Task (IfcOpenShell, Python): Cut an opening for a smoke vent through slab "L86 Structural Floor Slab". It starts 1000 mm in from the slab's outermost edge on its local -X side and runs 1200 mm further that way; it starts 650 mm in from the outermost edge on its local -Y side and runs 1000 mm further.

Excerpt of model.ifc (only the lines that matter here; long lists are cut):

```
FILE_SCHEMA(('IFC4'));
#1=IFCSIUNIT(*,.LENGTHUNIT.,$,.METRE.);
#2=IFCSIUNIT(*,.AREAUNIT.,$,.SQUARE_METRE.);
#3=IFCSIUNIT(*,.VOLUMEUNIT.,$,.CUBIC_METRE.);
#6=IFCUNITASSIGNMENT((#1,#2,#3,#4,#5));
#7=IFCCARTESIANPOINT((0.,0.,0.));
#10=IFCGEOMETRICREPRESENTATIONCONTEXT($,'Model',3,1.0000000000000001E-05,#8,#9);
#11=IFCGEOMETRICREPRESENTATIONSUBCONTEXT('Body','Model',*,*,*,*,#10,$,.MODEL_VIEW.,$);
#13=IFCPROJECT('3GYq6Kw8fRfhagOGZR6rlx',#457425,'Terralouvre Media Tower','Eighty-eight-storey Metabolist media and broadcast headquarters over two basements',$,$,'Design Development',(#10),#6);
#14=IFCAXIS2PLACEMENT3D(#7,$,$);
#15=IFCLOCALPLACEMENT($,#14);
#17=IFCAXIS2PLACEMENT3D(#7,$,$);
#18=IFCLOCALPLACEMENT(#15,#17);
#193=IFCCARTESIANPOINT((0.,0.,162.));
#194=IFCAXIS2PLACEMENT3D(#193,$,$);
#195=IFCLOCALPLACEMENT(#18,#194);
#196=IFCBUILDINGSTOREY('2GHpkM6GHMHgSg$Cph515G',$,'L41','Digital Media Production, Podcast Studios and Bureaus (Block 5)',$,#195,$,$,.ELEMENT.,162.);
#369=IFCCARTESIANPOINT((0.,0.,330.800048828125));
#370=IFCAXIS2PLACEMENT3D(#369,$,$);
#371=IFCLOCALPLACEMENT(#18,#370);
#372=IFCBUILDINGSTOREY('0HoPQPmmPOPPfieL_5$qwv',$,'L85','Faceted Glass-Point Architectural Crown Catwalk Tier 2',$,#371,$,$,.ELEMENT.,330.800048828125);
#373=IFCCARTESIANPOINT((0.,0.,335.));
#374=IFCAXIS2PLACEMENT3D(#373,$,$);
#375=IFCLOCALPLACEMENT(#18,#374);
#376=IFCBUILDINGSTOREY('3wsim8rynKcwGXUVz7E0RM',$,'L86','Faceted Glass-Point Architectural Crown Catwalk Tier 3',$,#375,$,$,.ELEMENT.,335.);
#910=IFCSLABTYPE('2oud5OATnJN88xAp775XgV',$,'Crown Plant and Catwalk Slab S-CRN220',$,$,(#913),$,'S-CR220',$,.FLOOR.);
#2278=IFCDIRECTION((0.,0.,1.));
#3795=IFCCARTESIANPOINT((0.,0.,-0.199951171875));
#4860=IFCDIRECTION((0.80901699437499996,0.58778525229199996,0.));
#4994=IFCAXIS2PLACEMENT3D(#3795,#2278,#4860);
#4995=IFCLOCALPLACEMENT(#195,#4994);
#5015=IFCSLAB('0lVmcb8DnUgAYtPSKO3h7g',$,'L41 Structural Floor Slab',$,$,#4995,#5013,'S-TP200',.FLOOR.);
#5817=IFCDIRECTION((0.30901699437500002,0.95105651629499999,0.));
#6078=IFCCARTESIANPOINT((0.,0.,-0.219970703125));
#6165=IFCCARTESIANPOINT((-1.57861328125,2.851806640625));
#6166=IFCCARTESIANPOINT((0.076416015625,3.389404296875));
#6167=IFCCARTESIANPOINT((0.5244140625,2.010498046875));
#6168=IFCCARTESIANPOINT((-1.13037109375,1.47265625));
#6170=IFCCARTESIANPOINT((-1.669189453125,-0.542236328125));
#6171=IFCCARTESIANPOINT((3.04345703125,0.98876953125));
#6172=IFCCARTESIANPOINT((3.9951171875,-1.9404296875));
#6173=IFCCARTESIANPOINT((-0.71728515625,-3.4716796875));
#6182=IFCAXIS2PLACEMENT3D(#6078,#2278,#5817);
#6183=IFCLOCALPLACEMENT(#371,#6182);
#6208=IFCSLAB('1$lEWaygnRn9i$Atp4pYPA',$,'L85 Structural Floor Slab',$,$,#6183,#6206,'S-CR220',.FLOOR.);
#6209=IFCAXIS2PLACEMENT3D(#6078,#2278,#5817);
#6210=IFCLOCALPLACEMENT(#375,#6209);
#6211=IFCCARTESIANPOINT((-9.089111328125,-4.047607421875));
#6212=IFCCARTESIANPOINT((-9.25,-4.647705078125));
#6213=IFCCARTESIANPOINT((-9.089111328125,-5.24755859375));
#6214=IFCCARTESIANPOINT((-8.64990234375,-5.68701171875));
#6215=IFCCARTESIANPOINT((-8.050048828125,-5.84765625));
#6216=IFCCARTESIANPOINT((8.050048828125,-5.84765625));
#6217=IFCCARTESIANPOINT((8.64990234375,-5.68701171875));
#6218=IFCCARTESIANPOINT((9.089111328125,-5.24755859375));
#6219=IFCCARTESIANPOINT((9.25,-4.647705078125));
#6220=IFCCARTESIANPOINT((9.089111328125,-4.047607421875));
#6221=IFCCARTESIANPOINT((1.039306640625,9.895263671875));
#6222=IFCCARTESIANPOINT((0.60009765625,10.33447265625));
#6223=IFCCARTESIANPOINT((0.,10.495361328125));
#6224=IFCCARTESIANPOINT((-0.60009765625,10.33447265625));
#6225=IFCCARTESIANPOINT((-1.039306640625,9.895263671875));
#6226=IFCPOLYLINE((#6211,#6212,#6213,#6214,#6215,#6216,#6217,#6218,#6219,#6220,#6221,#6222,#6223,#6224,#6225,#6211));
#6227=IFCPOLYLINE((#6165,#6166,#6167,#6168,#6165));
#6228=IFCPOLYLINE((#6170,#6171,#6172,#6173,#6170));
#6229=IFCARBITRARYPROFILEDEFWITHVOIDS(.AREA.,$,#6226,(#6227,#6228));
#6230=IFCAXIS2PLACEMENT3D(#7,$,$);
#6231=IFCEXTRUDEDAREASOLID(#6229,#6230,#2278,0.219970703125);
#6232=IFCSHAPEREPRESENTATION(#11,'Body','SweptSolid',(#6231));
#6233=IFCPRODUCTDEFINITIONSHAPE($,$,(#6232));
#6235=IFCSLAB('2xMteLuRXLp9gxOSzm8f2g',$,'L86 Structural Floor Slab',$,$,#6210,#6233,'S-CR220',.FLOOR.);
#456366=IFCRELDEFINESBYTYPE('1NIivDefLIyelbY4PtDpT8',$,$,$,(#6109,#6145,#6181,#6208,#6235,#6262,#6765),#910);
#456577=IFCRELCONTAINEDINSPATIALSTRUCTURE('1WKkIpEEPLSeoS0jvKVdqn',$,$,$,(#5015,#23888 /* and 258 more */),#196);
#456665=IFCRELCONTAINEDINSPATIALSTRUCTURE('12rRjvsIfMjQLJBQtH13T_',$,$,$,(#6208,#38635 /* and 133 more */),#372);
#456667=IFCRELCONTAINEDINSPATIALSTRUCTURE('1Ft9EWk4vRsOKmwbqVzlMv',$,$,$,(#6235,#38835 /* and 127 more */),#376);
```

```python
import numpy as np
import ifcopenshell
import ifcopenshell.api.feature
import ifcopenshell.api.geometry
import ifcopenshell.api.root
import ifcopenshell.geom
import ifcopenshell.util.placement
import ifcopenshell.util.representation
import ifcopenshell.util.shape
import ifcopenshell.util.unit

model = ifcopenshell.open("model.ifc")
unit_scale = ifcopenshell.util.unit.calculate_unit_scale(model)
settings = ifcopenshell.geom.settings()


def volume(element):
    """Net volume in cubic metres, openings subtracted."""
    shape = ifcopenshell.geom.create_shape(settings, element)
    return ifcopenshell.util.shape.get_volume(shape.geometry)


slab = model.by_id(6235)
before = volume(slab)

# Extent in the slab's own axes, in metres. The edges named are its -X and -Y sides.
slab_shape = ifcopenshell.geom.create_shape(settings, slab)
vertices = ifcopenshell.util.shape.get_vertices(slab_shape.geometry)
x_min, y_min, bottom = vertices.min(axis=0)
top = vertices[:, 2].max()

opening = ifcopenshell.api.root.create_entity(model, ifc_class="IfcOpeningElement", name="Smoke vent opening", predefined_type="OPENING")
context = ifcopenshell.util.representation.get_context(model, "Model", "Body", "MODEL_VIEW")
width, depth = 1.2, 1
outline = [(0.0, 0.0), (width, 0.0), (width, depth), (0.0, depth), (0.0, 0.0)]
# Overshoot both faces by 50 mm so the cut is clean.
shape = ifcopenshell.api.geometry.add_slab_representation(
    model, context=context, depth=top - bottom + 0.1, polyline=outline
)
ifcopenshell.api.geometry.assign_representation(model, product=opening, representation=shape)

matrix = ifcopenshell.util.placement.get_local_placement(slab.ObjectPlacement)
matrix[:, 3] = matrix @ np.append(np.array([x_min + 1, y_min + 0.65, bottom - 0.05]) / unit_scale, 1.0)
ifcopenshell.api.geometry.edit_object_placement(model, product=opening, matrix=matrix, is_si=False)
ifcopenshell.api.feature.add_feature(model, feature=opening, element=slab)

after = volume(slab)

print(f"slab volume {before:.3f} -> {after:.3f} m3")

model.write("model_updated.ifc")
```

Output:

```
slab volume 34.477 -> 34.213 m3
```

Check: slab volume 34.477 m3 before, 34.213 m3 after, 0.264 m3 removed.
